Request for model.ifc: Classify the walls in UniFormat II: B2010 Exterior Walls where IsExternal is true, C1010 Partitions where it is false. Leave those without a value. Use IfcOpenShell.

First a look at what the model holds.

```python
import ifcopenshell
import ifcopenshell.util.element

model = ifcopenshell.open("model.ifc")
print(model.schema)
print("classifications:", [c.Name for c in model.by_type("IfcClassification")])
values = [ifcopenshell.util.element.get_pset(e, "Pset_WallCommon", "IsExternal") for e in model.by_type("IfcWall")]
for value in (True, False, None):
    print("IsExternal", value, values.count(value))
```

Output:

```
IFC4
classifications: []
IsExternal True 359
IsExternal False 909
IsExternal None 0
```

```python
import ifcopenshell
import ifcopenshell.api.classification
import ifcopenshell.util.element

model = ifcopenshell.open("model.ifc")

system = ifcopenshell.api.classification.add_classification(model, classification="UniFormat II")

walls = model.by_type("IfcWall")
external = {e: ifcopenshell.util.element.get_pset(e, "Pset_WallCommon", "IsExternal") for e in walls}
for flag, code, name in ((True, "B2010", "Exterior Walls"), (False, "C1010", "Partitions")):
    products = [e for e in walls if external[e] is flag]
    ifcopenshell.api.classification.add_reference(
        model, products=products, classification=system, identification=code, name=name
    )
    print(code, len(products))

model.write("model_updated.ifc")
```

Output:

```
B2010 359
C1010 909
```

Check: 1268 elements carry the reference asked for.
